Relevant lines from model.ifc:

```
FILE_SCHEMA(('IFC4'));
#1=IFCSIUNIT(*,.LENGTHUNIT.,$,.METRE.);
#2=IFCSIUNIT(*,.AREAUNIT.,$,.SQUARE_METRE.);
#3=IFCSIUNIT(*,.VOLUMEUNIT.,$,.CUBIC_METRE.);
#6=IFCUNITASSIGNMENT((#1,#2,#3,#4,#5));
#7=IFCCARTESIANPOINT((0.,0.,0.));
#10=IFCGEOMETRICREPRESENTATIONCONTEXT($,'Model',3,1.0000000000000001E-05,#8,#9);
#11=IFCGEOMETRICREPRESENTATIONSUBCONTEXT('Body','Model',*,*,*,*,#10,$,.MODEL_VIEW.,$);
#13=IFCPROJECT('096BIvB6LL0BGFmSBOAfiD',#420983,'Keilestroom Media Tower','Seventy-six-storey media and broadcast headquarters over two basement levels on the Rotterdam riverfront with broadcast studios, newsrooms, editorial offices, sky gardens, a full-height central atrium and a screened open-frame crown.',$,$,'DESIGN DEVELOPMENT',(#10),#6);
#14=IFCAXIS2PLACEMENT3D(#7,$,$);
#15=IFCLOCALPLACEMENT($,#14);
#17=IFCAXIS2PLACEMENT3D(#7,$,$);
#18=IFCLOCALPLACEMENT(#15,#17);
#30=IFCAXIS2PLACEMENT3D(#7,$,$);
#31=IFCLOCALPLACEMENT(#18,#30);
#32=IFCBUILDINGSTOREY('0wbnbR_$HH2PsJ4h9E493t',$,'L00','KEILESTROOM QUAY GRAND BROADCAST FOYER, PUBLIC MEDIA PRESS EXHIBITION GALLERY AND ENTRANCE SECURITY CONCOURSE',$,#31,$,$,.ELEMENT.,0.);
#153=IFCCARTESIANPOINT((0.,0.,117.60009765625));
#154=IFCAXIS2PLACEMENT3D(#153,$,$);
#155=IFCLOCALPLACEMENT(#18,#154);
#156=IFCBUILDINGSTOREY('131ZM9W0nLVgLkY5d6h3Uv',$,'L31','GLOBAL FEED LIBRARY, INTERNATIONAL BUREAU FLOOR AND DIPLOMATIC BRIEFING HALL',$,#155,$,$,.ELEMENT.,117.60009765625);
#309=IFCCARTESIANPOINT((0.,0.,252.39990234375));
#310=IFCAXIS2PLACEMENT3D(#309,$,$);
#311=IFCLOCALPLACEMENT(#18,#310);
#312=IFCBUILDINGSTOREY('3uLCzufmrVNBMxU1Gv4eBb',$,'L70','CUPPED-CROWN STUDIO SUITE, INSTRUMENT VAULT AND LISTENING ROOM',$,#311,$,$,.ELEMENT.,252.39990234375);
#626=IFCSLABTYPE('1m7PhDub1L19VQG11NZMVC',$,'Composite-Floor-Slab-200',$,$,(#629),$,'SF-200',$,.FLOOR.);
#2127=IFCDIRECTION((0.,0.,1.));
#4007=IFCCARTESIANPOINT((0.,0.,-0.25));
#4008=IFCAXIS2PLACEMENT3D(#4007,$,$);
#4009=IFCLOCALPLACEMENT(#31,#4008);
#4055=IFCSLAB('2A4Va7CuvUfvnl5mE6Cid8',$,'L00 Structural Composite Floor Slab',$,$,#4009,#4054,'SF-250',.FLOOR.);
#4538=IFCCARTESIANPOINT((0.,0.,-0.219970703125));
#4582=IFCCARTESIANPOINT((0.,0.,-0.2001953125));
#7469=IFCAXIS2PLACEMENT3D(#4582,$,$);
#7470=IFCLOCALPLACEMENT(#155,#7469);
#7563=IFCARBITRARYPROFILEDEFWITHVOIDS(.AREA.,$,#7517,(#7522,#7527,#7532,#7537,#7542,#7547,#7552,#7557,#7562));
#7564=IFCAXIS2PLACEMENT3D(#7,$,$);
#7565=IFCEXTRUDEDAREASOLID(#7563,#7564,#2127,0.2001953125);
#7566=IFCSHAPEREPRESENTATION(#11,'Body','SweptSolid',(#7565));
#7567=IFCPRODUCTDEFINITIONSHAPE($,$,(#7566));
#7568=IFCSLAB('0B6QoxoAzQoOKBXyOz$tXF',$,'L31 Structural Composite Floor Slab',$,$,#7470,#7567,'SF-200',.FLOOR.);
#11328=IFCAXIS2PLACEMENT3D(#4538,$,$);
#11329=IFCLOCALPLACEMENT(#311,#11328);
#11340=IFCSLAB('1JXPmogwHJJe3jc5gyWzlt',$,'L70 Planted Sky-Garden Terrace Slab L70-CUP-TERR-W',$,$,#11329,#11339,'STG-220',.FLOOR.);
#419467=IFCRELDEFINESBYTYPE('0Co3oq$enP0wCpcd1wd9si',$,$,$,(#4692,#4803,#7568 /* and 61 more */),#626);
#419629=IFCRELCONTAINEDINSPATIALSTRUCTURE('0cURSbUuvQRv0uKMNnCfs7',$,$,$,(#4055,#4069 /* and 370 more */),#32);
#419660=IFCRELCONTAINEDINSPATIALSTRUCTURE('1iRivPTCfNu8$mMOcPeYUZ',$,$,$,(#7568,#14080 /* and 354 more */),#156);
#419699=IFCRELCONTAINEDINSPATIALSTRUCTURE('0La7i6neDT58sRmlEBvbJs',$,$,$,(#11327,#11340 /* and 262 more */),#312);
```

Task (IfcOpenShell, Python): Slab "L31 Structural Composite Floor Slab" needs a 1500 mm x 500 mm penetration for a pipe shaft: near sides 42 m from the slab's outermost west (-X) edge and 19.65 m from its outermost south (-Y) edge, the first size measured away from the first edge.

```python
import numpy as np
import ifcopenshell
import ifcopenshell.api.feature
import ifcopenshell.api.geometry
import ifcopenshell.api.root
import ifcopenshell.geom
import ifcopenshell.util.placement
import ifcopenshell.util.representation
import ifcopenshell.util.shape
import ifcopenshell.util.unit

model = ifcopenshell.open("model.ifc")
unit_scale = ifcopenshell.util.unit.calculate_unit_scale(model)
settings = ifcopenshell.geom.settings()


def volume(element):
    """Net volume in cubic metres, openings subtracted."""
    shape = ifcopenshell.geom.create_shape(settings, element)
    return ifcopenshell.util.shape.get_volume(shape.geometry)


slab = model.by_id(7568)
before = volume(slab)

# Extent in the slab's own axes, in metres. The edges named are its -X and -Y sides.
slab_shape = ifcopenshell.geom.create_shape(settings, slab)
vertices = ifcopenshell.util.shape.get_vertices(slab_shape.geometry)
x_min, y_min, bottom = vertices.min(axis=0)
top = vertices[:, 2].max()

opening = ifcopenshell.api.root.create_entity(model, ifc_class="IfcOpeningElement", name="Pipe shaft opening", predefined_type="OPENING")
context = ifcopenshell.util.representation.get_context(model, "Model", "Body", "MODEL_VIEW")
width, depth = 1.5, 0.5
outline = [(0.0, 0.0), (width, 0.0), (width, depth), (0.0, depth), (0.0, 0.0)]
# Overshoot both faces by 50 mm so the cut is clean.
shape = ifcopenshell.api.geometry.add_slab_representation(
    model, context=context, depth=top - bottom + 0.1, polyline=outline
)
ifcopenshell.api.geometry.assign_representation(model, product=opening, representation=shape)

matrix = ifcopenshell.util.placement.get_local_placement(slab.ObjectPlacement)
matrix[:, 3] = matrix @ np.append(np.array([x_min + 42, y_min + 19.65, bottom - 0.05]) / unit_scale, 1.0)
ifcopenshell.api.geometry.edit_object_placement(model, product=opening, matrix=matrix, is_si=False)
ifcopenshell.api.feature.add_feature(model, feature=opening, element=slab)

after = volume(slab)

print(f"slab volume {before:.3f} -> {after:.3f} m3")

model.write("model_v2.ifc")
```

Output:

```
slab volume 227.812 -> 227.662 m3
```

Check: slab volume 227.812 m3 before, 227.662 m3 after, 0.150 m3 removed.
